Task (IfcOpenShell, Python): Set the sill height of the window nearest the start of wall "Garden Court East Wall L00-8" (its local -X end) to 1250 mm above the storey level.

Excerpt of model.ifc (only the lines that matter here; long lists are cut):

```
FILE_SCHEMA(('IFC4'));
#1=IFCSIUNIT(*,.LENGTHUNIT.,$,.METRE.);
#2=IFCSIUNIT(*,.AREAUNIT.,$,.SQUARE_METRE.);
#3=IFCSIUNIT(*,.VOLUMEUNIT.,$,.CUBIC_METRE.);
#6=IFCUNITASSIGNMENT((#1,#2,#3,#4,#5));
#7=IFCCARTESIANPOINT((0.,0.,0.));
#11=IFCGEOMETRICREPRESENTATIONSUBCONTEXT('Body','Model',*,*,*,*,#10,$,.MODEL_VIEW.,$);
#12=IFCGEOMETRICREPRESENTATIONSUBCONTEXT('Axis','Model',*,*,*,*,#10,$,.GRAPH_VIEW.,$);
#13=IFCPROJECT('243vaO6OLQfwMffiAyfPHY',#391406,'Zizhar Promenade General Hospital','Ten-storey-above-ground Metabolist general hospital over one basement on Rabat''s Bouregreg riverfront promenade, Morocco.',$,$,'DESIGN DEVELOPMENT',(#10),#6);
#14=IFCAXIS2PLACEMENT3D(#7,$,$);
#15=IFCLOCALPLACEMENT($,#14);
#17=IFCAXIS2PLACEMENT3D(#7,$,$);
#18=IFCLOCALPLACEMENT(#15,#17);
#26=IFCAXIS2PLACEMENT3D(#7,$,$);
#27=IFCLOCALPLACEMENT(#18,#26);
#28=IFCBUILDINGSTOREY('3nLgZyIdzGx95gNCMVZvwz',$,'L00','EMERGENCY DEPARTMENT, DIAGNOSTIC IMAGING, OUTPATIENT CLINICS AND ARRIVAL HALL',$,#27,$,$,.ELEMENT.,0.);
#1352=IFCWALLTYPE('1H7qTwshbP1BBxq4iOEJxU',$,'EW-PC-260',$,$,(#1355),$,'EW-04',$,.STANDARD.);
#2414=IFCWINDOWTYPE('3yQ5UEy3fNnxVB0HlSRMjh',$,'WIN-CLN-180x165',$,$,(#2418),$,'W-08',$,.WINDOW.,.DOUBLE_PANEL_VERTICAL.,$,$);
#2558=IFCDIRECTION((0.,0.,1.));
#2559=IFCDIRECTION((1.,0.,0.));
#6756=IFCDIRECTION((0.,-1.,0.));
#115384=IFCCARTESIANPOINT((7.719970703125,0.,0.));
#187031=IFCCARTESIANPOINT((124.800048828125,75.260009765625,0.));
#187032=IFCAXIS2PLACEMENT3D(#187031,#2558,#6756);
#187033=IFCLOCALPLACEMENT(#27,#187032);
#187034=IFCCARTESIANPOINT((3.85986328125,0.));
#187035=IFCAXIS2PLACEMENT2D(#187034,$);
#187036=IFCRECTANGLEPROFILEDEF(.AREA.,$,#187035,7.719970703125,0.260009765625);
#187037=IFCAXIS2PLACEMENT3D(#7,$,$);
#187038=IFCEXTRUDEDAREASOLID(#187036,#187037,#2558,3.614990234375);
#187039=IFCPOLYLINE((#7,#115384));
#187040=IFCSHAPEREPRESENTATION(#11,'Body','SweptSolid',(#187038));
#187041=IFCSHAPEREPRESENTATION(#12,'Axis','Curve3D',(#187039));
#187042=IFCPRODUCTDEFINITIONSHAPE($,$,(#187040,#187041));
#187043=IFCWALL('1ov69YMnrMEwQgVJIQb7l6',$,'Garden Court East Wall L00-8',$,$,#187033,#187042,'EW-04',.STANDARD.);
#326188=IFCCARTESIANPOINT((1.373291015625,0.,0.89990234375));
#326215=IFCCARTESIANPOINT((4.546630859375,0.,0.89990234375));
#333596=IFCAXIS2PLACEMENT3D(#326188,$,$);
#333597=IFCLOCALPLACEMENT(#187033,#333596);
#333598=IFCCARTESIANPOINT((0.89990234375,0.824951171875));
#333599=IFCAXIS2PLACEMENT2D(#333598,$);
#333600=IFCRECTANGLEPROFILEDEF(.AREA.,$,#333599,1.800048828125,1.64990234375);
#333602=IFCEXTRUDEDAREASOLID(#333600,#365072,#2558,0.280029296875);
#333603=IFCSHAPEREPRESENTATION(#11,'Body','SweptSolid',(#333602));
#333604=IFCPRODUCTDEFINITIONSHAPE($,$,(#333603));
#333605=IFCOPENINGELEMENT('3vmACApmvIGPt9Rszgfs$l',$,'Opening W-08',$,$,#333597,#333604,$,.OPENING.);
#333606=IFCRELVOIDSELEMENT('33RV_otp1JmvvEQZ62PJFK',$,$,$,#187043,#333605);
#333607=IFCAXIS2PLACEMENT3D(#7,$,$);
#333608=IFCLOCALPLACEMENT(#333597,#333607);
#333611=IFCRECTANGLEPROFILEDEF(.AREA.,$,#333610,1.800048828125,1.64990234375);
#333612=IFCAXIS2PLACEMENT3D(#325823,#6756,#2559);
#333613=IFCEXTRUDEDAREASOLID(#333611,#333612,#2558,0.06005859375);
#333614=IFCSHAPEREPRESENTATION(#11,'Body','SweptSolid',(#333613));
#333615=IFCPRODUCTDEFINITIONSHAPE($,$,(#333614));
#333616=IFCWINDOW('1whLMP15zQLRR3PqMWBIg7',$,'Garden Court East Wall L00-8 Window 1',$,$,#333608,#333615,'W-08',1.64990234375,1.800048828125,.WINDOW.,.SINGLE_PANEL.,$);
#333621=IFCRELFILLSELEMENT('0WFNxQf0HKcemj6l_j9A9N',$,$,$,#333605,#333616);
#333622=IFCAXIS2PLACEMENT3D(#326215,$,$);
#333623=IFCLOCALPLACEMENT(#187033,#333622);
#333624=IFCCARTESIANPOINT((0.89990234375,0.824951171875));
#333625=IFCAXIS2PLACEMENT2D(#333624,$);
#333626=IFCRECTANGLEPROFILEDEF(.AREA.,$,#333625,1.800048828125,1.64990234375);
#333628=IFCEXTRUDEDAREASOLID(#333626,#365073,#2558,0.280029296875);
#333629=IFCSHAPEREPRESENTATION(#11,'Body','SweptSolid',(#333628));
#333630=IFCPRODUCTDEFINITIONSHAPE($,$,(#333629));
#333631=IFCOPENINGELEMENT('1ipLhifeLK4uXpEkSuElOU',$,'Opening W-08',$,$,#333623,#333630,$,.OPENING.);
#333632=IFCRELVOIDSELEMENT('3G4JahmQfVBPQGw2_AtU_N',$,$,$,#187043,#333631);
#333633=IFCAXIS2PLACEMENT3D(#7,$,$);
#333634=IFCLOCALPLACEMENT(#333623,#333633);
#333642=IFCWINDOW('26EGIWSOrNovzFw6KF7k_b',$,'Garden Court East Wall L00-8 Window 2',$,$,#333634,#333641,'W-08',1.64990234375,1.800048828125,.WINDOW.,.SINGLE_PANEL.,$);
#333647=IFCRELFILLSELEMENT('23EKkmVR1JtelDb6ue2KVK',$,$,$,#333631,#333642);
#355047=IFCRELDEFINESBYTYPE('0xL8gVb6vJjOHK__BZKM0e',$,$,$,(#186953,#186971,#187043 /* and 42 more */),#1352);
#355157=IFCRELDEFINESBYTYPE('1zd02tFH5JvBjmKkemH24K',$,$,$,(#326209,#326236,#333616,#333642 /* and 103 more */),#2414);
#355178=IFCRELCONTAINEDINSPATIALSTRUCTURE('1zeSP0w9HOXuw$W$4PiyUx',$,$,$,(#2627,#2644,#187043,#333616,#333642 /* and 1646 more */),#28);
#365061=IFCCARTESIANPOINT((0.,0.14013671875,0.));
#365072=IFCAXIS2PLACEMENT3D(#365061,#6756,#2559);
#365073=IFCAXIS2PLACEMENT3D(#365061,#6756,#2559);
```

```python
import numpy as np
import ifcopenshell
import ifcopenshell.api.geometry
import ifcopenshell.geom
import ifcopenshell.util.element
import ifcopenshell.util.placement
import ifcopenshell.util.shape
import ifcopenshell.util.unit

model = ifcopenshell.open("model.ifc")
unit_scale = ifcopenshell.util.unit.calculate_unit_scale(model)

window = model.by_guid("1whLMP15zQLRR3PqMWBIg7")
opening = window.FillsVoids[0].RelatingOpeningElement
storey = ifcopenshell.util.element.get_container(window, ifc_class="IfcBuildingStorey")
level = ifcopenshell.util.placement.get_local_placement(storey.ObjectPlacement)[2, 3]

# The opening's origin need not be at the sill, so measure its lowest point.
shape = ifcopenshell.geom.create_shape(ifcopenshell.geom.settings(), opening)
bottom = ifcopenshell.util.shape.get_shape_bottom_elevation(shape, shape.geometry) / unit_scale
dz = level + 1.25 / unit_scale - bottom

shift = np.array([0.0, 0.0, dz])
# The window is placed relative to its opening, so it follows when the opening moves.
matrix = ifcopenshell.util.placement.get_local_placement(opening.ObjectPlacement)
matrix[:3, 3] += shift
ifcopenshell.api.geometry.edit_object_placement(
    model, product=opening, matrix=matrix, is_si=False, should_transform_children=True
)

print(f"moved by {dz * unit_scale:+.3f} m")

model.write("model-out.ifc")
```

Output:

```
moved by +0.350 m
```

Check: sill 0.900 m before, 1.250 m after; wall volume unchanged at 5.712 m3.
